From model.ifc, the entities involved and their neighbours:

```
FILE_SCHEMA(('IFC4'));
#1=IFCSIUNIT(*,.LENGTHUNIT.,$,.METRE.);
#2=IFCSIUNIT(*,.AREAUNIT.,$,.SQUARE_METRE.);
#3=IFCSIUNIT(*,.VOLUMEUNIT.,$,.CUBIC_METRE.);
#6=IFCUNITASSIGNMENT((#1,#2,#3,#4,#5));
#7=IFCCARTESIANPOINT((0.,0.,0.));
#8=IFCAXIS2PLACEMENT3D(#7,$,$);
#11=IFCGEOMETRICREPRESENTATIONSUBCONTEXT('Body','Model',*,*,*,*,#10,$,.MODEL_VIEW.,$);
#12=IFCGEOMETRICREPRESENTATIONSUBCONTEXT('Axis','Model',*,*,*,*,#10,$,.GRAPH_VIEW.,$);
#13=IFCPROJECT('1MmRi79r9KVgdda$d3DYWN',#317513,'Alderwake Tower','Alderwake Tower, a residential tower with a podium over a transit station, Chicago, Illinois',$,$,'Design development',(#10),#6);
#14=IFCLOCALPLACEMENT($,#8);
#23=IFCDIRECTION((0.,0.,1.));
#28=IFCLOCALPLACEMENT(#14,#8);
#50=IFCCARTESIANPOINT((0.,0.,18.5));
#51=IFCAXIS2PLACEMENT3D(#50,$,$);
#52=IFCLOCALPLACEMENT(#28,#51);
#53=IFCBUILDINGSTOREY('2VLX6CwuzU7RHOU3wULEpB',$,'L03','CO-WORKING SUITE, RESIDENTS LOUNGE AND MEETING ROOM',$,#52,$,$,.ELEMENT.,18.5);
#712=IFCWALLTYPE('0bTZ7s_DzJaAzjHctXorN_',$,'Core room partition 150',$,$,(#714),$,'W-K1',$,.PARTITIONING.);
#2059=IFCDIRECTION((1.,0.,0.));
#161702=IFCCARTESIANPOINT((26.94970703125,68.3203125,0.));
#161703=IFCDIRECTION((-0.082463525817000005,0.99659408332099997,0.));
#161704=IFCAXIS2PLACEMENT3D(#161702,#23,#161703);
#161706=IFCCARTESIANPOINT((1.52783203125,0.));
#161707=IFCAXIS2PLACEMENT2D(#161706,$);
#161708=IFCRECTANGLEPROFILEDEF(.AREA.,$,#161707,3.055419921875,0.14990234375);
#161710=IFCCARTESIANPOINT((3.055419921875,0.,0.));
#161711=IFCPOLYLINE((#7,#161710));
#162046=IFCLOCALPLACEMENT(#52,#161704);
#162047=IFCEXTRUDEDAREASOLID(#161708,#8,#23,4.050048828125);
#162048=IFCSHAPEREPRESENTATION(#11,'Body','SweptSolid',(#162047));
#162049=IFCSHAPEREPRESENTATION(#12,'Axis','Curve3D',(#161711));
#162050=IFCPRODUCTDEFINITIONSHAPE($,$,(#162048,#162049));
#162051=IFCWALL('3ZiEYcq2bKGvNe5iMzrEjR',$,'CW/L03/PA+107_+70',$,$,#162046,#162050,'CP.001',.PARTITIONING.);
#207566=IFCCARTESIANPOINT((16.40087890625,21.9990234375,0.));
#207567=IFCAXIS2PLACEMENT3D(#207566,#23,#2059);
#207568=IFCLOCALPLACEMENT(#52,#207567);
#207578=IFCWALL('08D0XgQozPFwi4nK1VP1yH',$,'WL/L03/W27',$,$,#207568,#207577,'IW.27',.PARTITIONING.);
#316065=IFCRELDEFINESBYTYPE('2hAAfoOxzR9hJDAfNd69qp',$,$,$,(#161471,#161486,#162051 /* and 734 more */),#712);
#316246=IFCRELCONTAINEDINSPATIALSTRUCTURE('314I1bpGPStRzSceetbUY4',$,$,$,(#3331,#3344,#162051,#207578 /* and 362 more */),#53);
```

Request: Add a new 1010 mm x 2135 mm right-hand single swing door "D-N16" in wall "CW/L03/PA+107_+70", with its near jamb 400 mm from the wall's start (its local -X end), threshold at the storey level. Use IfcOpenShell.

```python
import numpy as np
import ifcopenshell
import ifcopenshell.api.feature
import ifcopenshell.api.geometry
import ifcopenshell.api.root
import ifcopenshell.api.spatial
import ifcopenshell.geom
import ifcopenshell.util.element
import ifcopenshell.util.placement
import ifcopenshell.util.representation
import ifcopenshell.util.shape
import ifcopenshell.util.unit

model = ifcopenshell.open("model.ifc")
unit_scale = ifcopenshell.util.unit.calculate_unit_scale(model)
settings = ifcopenshell.geom.settings()


def volume(element):
    """Net volume in cubic metres, openings subtracted."""
    shape = ifcopenshell.geom.create_shape(settings, element)
    return ifcopenshell.util.shape.get_volume(shape.geometry)


wall = model.by_guid("3ZiEYcq2bKGvNe5iMzrEjR")
storey = ifcopenshell.util.element.get_container(wall, ifc_class="IfcBuildingStorey")
context = ifcopenshell.util.representation.get_context(model, "Model", "Body", "MODEL_VIEW")
before = volume(wall)

width, height, from_end, sill = 1.01, 2.135, 0.4, 0.0  # metres

# The wall runs along its own X axis, and the end named is its -X end.
wall_shape = ifcopenshell.geom.create_shape(settings, wall)
x, y, z = ifcopenshell.util.shape.get_vertices(wall_shape.geometry).T
start = x.min() + from_end
face, thickness = float(y.min()), float(y.max() - y.min())
wall_matrix = ifcopenshell.util.placement.get_local_placement(wall.ObjectPlacement)
level = ifcopenshell.util.placement.get_local_placement(storey.ObjectPlacement)[2, 3]


def in_wall(x, y):
    """Placement at x, y metres in the wall's axes, at sill height."""
    matrix = wall_matrix.copy()
    matrix[:, 3] = wall_matrix @ np.array([x / unit_scale, y / unit_scale, 0.0, 1.0])
    matrix[2, 3] = level + sill / unit_scale
    return matrix


# Opening: a box that overshoots both wall faces by 50 mm.
opening = ifcopenshell.api.root.create_entity(model, ifc_class="IfcOpeningElement", predefined_type="OPENING")
box = ifcopenshell.api.geometry.add_wall_representation(
    model, context=context, length=width, height=height, thickness=thickness + 0.1
)
ifcopenshell.api.geometry.assign_representation(model, product=opening, representation=box)
ifcopenshell.api.geometry.edit_object_placement(model, product=opening, matrix=in_wall(start, face - 0.05), is_si=False)
ifcopenshell.api.feature.add_feature(model, feature=opening, element=wall)

door = ifcopenshell.api.root.create_entity(model, ifc_class="IfcDoor", name="D-N16", predefined_type="DOOR")
door.OverallWidth, door.OverallHeight = width / unit_scale, height / unit_scale
door.OperationType = "SINGLE_SWING_RIGHT"
body = ifcopenshell.api.geometry.add_door_representation(
    model,
    context=context,
    overall_width=door.OverallWidth,
    overall_height=door.OverallHeight,
    operation_type="SINGLE_SWING_RIGHT",
    lining_properties={"LiningDepth": thickness / unit_scale, "ThresholdDepth": thickness / unit_scale},
)
ifcopenshell.api.geometry.assign_representation(model, product=door, representation=body)
ifcopenshell.api.spatial.assign_container(model, products=[door], relating_structure=storey)
ifcopenshell.api.feature.add_filling(model, opening=opening, element=door)

# The lining spans the wall, so the door starts at the wall face.
ifcopenshell.api.geometry.edit_object_placement(model, product=door, matrix=in_wall(start, face), is_si=False)

after = volume(wall)

print(f"wall volume {before:.3f} -> {after:.3f} m3")

model.write("model_v2.ifc")
```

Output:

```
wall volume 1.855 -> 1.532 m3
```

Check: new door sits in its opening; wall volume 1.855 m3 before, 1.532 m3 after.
